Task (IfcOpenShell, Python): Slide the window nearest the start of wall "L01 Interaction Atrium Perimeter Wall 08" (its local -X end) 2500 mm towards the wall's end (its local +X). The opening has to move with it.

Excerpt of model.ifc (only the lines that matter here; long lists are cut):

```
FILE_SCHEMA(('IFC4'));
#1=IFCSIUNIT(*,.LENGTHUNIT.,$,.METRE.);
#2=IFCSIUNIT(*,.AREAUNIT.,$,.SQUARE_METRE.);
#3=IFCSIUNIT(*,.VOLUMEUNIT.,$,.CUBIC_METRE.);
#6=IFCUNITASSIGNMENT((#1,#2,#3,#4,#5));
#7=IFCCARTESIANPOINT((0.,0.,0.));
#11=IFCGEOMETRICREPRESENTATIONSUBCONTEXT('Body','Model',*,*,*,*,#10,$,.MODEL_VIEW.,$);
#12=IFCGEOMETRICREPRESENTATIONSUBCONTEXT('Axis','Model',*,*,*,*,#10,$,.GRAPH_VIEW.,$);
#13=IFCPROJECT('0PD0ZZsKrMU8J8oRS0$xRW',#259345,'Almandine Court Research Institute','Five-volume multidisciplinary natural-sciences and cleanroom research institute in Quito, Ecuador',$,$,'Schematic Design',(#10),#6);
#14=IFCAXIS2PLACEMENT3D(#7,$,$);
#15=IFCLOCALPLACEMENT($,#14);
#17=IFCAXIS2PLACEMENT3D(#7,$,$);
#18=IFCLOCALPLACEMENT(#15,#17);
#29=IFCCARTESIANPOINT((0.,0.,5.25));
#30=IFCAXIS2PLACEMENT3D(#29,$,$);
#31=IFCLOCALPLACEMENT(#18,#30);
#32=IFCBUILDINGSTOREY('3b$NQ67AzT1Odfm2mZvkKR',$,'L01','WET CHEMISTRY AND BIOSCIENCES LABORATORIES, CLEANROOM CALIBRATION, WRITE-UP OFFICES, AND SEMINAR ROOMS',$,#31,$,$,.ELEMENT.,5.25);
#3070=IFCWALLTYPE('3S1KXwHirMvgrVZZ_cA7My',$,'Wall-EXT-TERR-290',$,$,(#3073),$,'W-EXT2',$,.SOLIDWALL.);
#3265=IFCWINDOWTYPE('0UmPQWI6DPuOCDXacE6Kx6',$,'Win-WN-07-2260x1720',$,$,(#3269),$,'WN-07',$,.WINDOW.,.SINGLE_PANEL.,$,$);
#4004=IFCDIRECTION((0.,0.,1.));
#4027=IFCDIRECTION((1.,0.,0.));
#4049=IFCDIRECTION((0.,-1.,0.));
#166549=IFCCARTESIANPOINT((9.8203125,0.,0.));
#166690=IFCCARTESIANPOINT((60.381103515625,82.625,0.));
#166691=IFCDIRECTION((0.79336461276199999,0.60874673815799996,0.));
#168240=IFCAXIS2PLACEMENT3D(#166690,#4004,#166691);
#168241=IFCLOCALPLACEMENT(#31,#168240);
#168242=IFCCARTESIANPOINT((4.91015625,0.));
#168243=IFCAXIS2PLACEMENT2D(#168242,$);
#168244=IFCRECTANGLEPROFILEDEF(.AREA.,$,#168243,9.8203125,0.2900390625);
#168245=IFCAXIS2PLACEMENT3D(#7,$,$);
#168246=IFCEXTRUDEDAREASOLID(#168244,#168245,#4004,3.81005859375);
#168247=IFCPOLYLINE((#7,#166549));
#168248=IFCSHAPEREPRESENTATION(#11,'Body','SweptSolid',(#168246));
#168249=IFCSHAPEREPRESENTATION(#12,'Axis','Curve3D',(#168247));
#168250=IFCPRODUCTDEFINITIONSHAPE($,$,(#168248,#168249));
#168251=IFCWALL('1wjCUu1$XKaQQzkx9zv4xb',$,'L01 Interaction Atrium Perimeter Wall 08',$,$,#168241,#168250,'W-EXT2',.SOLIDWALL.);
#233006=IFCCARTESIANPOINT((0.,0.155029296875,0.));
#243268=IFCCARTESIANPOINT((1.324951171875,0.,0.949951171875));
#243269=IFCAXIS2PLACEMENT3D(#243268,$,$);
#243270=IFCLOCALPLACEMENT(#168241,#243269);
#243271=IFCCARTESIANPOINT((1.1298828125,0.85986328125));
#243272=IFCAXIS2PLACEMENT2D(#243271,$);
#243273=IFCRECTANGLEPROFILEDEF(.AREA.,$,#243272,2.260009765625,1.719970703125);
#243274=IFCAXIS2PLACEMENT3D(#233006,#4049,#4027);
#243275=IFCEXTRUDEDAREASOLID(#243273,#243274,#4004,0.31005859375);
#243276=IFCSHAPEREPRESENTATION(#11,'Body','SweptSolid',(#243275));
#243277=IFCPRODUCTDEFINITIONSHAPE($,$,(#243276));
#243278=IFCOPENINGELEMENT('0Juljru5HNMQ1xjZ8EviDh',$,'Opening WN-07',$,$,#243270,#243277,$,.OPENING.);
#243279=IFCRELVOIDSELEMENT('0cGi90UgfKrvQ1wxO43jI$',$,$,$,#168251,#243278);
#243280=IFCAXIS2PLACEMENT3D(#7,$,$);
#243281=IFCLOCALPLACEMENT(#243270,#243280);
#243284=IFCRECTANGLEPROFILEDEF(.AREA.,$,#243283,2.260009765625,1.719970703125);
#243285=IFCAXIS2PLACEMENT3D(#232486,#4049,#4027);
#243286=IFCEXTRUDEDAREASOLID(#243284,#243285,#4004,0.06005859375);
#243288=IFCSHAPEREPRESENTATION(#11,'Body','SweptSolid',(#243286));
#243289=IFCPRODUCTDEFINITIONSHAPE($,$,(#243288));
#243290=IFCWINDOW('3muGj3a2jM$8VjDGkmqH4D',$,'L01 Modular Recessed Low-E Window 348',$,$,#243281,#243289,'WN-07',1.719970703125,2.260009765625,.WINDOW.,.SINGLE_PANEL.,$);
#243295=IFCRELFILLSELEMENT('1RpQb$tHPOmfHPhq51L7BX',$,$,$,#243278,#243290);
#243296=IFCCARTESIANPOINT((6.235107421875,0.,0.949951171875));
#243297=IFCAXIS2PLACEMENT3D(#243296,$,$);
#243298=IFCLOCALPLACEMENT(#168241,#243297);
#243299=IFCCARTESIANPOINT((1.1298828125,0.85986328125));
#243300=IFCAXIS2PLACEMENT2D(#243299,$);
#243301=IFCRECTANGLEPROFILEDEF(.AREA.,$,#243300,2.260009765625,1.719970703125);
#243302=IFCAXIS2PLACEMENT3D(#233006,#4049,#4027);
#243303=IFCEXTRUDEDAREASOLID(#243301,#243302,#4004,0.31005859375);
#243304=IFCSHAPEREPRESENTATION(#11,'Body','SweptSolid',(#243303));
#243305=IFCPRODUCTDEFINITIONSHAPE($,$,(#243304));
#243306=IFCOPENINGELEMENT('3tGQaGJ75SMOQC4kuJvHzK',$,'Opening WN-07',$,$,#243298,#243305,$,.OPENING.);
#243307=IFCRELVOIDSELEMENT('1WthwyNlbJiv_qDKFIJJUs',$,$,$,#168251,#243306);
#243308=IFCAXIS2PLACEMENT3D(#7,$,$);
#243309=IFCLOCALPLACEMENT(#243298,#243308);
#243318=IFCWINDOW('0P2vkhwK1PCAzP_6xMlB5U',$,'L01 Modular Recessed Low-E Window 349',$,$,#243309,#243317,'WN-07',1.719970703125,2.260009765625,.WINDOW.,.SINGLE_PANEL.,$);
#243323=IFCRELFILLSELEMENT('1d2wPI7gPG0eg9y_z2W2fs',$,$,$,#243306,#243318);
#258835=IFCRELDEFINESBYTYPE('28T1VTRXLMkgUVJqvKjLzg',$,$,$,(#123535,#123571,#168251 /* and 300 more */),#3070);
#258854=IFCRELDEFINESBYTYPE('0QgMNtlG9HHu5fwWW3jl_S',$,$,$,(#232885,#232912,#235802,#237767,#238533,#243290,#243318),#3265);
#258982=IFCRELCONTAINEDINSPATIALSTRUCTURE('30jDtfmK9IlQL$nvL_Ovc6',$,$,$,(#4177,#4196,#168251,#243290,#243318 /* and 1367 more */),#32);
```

```python
import ifcopenshell
import ifcopenshell.api.geometry
import ifcopenshell.util.placement
import ifcopenshell.util.unit

model = ifcopenshell.open("model.ifc")
unit_scale = ifcopenshell.util.unit.calculate_unit_scale(model)

window = model.by_guid("3muGj3a2jM$8VjDGkmqH4D")
opening = window.FillsVoids[0].RelatingOpeningElement
wall = opening.VoidsElements[0].RelatingBuildingElement

wall_matrix = ifcopenshell.util.placement.get_local_placement(wall.ObjectPlacement)
shift = wall_matrix[:3, 0] * 2.5 / unit_scale
before = ifcopenshell.util.placement.get_local_placement(window.ObjectPlacement)[:3, 3].copy()

# The window is placed relative to its opening, so it follows when the opening moves.
matrix = ifcopenshell.util.placement.get_local_placement(opening.ObjectPlacement)
matrix[:3, 3] += shift
ifcopenshell.api.geometry.edit_object_placement(
    model, product=opening, matrix=matrix, is_si=False, should_transform_children=True
)

after = ifcopenshell.util.placement.get_local_placement(window.ObjectPlacement)[:3, 3]
print("window moved by", (after - before).round(3) + 0.0)

model.write("model_edited.ifc")
```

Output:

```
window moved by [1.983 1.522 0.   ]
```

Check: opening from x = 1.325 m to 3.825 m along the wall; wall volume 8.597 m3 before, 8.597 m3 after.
